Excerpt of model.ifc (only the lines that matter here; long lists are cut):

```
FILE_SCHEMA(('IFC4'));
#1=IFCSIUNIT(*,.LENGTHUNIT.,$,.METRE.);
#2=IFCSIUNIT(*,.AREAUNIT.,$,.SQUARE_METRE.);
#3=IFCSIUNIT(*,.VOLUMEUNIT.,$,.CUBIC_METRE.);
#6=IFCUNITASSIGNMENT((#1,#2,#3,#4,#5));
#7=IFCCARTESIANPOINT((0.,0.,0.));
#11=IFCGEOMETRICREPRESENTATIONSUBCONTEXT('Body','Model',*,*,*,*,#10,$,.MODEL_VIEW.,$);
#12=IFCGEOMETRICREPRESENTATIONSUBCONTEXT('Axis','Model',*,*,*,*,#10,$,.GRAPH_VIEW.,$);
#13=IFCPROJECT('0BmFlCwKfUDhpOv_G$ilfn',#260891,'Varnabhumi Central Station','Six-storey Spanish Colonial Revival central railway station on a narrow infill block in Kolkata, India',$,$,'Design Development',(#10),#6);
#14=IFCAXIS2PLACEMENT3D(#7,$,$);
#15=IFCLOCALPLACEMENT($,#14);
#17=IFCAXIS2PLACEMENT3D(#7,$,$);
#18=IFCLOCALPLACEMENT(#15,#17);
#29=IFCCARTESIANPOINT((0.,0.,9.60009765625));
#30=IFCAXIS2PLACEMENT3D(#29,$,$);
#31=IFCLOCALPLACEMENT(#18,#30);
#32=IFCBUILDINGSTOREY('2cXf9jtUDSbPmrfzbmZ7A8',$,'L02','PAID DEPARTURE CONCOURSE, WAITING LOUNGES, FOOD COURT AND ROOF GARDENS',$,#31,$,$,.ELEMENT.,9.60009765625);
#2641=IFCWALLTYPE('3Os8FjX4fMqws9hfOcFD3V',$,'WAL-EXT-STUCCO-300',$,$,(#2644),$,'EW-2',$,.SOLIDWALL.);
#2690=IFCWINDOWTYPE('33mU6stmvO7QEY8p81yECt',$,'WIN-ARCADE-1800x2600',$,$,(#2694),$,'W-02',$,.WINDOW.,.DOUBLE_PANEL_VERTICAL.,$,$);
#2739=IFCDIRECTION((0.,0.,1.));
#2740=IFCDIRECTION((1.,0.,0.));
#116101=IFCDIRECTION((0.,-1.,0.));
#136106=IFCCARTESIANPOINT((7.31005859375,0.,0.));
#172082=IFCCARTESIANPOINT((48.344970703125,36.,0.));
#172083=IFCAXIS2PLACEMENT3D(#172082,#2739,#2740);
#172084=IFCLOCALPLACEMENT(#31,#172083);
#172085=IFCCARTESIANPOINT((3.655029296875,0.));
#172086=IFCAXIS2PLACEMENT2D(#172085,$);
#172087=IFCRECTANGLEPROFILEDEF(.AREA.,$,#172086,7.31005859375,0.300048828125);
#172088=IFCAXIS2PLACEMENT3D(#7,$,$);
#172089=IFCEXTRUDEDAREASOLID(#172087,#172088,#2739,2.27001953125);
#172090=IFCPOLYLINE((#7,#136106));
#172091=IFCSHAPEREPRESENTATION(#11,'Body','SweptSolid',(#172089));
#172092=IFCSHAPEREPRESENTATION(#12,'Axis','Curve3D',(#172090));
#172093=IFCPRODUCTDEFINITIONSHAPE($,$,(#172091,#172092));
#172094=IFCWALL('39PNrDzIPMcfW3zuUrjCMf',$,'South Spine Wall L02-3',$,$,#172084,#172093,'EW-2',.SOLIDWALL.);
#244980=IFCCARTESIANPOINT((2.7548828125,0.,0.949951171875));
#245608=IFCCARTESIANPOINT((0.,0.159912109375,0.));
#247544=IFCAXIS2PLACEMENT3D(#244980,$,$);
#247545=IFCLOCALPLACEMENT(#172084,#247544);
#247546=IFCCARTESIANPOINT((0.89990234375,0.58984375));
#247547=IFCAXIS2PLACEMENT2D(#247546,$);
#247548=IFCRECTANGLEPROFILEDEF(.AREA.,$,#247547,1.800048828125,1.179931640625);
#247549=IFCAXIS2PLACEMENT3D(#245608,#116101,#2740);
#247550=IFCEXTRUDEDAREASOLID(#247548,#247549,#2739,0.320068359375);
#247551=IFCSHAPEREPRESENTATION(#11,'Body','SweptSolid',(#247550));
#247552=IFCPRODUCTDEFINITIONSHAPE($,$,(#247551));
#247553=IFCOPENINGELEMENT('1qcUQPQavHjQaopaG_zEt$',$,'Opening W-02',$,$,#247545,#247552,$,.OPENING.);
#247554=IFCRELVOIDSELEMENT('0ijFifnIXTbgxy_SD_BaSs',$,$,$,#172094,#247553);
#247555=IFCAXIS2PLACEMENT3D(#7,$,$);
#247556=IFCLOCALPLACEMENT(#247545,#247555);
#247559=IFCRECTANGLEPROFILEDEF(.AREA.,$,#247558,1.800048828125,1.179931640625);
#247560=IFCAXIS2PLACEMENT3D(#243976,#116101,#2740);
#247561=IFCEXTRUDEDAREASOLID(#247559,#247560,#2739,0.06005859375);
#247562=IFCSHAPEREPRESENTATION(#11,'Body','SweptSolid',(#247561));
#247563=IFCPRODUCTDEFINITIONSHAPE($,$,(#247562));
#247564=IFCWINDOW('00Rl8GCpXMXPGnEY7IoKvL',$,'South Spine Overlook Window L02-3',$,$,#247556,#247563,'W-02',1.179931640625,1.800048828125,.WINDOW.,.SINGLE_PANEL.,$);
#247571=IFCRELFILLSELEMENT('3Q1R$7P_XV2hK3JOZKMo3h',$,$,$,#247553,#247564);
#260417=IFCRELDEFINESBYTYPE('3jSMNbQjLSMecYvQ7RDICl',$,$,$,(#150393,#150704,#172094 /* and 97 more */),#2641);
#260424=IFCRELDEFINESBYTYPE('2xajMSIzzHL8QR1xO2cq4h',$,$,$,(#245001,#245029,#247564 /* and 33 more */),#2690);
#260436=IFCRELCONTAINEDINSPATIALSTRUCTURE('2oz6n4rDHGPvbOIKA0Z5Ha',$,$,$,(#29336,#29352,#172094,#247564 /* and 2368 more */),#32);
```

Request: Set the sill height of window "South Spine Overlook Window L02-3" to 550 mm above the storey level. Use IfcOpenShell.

```python
import numpy as np
import ifcopenshell
import ifcopenshell.api.geometry
import ifcopenshell.geom
import ifcopenshell.util.element
import ifcopenshell.util.placement
import ifcopenshell.util.shape
import ifcopenshell.util.unit

model = ifcopenshell.open("model.ifc")
unit_scale = ifcopenshell.util.unit.calculate_unit_scale(model)

window = model.by_guid("00Rl8GCpXMXPGnEY7IoKvL")
opening = window.FillsVoids[0].RelatingOpeningElement
storey = ifcopenshell.util.element.get_container(window, ifc_class="IfcBuildingStorey")
level = ifcopenshell.util.placement.get_local_placement(storey.ObjectPlacement)[2, 3]

# The opening's origin need not be at the sill, so measure its lowest point.
shape = ifcopenshell.geom.create_shape(ifcopenshell.geom.settings(), opening)
bottom = ifcopenshell.util.shape.get_shape_bottom_elevation(shape, shape.geometry) / unit_scale
dz = level + 0.55 / unit_scale - bottom

shift = np.array([0.0, 0.0, dz])
# The window is placed relative to its opening, so it follows when the opening moves.
matrix = ifcopenshell.util.placement.get_local_placement(opening.ObjectPlacement)
matrix[:3, 3] += shift
ifcopenshell.api.geometry.edit_object_placement(
    model, product=opening, matrix=matrix, is_si=False, should_transform_children=True
)

print(f"moved by {dz * unit_scale:+.3f} m")

model.write("model_updated.ifc")
```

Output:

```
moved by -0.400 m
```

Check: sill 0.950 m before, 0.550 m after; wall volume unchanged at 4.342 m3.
